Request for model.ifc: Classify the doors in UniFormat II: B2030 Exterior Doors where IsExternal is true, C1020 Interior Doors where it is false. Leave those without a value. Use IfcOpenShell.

First a look at what the model holds.

```python
import ifcopenshell
import ifcopenshell.util.element

model = ifcopenshell.open("model.ifc")
print(model.schema)
print("classifications:", [c.Name for c in model.by_type("IfcClassification")])
values = [ifcopenshell.util.element.get_pset(e, "Pset_DoorCommon", "IsExternal") for e in model.by_type("IfcDoor")]
for value in (True, False, None):
    print("IsExternal", value, values.count(value))
```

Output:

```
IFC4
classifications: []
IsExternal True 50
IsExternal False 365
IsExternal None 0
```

```python
import ifcopenshell
import ifcopenshell.api.classification
import ifcopenshell.util.element

model = ifcopenshell.open("model.ifc")

system = ifcopenshell.api.classification.add_classification(model, classification="UniFormat II")

doors = model.by_type("IfcDoor")
external = {e: ifcopenshell.util.element.get_pset(e, "Pset_DoorCommon", "IsExternal") for e in doors}
for flag, code, name in ((True, "B2030", "Exterior Doors"), (False, "C1020", "Interior Doors")):
    products = [e for e in doors if external[e] is flag]
    ifcopenshell.api.classification.add_reference(
        model, products=products, classification=system, identification=code, name=name
    )
    print(code, len(products))

model.write("model_updated.ifc")
```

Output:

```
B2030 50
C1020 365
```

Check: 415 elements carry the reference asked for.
